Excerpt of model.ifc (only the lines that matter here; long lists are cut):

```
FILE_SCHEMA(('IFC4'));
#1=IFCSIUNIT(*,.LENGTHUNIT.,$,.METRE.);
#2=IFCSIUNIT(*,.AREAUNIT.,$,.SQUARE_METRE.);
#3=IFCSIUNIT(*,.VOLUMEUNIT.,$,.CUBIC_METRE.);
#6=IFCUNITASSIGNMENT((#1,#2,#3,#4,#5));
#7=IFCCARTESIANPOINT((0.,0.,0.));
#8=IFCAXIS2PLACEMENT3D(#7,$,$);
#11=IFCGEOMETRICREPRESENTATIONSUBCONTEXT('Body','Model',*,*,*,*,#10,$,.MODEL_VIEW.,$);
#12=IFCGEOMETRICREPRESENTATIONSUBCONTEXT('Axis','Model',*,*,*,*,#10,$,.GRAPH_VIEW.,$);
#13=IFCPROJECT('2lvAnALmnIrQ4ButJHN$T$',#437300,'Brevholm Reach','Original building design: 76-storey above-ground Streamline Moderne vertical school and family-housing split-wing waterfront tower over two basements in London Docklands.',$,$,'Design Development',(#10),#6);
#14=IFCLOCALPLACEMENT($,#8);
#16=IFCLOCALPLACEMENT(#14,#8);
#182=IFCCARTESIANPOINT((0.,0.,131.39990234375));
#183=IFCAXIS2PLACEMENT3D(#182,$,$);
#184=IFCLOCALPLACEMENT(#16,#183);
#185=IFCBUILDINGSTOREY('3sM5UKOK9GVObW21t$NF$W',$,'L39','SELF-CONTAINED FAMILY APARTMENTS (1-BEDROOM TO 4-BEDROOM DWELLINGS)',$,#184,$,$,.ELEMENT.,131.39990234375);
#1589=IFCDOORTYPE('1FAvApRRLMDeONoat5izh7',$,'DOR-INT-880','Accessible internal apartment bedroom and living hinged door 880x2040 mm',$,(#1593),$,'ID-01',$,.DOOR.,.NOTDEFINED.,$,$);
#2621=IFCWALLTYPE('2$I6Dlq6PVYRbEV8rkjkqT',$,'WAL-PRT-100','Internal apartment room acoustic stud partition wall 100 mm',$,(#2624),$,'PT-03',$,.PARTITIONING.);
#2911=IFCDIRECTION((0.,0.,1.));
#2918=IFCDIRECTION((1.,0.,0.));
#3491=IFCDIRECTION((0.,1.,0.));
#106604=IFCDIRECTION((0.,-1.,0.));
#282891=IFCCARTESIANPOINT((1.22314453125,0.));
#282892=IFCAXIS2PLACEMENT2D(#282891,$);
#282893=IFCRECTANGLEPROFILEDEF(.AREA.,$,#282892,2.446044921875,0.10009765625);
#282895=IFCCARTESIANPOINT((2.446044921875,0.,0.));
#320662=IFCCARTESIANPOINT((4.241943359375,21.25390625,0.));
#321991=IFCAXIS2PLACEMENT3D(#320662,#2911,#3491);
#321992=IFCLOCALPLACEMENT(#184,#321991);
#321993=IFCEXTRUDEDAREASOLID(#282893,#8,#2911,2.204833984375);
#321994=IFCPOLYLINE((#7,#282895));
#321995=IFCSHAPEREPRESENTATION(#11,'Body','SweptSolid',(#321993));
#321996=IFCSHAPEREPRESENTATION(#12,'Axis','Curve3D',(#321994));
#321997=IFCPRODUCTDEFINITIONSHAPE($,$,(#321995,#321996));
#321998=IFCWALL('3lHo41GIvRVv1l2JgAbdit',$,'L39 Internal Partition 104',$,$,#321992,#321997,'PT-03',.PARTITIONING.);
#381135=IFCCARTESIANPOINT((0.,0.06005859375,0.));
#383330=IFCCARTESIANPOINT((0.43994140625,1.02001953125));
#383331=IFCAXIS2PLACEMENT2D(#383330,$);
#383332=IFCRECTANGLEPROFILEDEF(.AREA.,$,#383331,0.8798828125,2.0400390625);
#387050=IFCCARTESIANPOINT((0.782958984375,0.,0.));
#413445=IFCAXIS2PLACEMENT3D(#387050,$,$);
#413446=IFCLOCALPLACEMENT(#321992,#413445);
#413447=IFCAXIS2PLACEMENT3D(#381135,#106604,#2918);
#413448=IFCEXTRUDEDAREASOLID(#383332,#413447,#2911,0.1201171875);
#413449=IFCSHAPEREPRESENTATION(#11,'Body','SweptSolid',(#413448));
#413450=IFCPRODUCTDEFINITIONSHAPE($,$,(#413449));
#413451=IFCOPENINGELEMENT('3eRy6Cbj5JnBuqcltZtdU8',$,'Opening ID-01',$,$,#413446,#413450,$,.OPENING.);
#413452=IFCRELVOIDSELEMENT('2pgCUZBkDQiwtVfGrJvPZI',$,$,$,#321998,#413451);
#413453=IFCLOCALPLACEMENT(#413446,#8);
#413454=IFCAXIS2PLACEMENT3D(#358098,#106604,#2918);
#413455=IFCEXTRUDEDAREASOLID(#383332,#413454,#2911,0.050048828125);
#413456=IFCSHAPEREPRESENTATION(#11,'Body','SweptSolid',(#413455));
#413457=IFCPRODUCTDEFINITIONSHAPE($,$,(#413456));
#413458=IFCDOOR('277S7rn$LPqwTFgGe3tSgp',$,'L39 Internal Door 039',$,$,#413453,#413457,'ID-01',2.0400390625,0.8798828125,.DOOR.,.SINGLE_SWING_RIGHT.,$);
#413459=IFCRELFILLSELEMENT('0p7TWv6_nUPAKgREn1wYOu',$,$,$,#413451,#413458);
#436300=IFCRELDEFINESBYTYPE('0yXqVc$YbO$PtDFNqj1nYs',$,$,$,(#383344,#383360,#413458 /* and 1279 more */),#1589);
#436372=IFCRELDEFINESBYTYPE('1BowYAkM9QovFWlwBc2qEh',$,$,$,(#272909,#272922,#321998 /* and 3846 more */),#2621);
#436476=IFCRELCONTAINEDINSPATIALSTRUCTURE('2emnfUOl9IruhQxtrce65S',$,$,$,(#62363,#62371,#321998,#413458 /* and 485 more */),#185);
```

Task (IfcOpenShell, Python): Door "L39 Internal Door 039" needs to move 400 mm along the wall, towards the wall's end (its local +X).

```python
import ifcopenshell
import ifcopenshell.api.geometry
import ifcopenshell.util.placement

model = ifcopenshell.open("model.ifc")

door = model.by_guid("277S7rn$LPqwTFgGe3tSgp")
opening = door.FillsVoids[0].RelatingOpeningElement
wall = opening.VoidsElements[0].RelatingBuildingElement

wall_matrix = ifcopenshell.util.placement.get_local_placement(wall.ObjectPlacement)
shift = wall_matrix[:3, 0] * 0.4
before = ifcopenshell.util.placement.get_local_placement(door.ObjectPlacement)[:3, 3].copy()

# The door is placed relative to its opening, so it follows when the opening moves.
matrix = ifcopenshell.util.placement.get_local_placement(opening.ObjectPlacement)
matrix[:3, 3] += shift
ifcopenshell.api.geometry.edit_object_placement(
    model, product=opening, matrix=matrix, is_si=False, should_transform_children=True
)

after = ifcopenshell.util.placement.get_local_placement(door.ObjectPlacement)[:3, 3]
print("door moved by", (after - before).round(3) + 0.0)

model.write("model_rev.ifc")
```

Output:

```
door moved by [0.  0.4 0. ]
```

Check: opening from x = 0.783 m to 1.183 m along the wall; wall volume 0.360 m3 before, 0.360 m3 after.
